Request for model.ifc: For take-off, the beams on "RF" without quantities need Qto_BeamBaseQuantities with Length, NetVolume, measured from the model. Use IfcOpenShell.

First a look at what the model holds.

```python
import ifcopenshell
import ifcopenshell.util.element
import ifcopenshell.util.unit

model = ifcopenshell.open("model.ifc")
print(model.schema)
for unit_type in ("LENGTHUNIT", "AREAUNIT", "VOLUMEUNIT"):
    print(unit_type, ifcopenshell.util.unit.calculate_unit_scale(model, unit_type))
storey = next(s for s in model.by_type("IfcBuildingStorey") if s.Name == "RF")
beams = [e for e in ifcopenshell.util.element.get_decomposition(storey) if e.is_a("IfcBeam")]
for e in sorted(beams, key=lambda e: e.id()):
    print(e.id(), e.is_a(), e.Name, list(ifcopenshell.util.element.get_psets(e, qtos_only=True)), sep=" | ")
```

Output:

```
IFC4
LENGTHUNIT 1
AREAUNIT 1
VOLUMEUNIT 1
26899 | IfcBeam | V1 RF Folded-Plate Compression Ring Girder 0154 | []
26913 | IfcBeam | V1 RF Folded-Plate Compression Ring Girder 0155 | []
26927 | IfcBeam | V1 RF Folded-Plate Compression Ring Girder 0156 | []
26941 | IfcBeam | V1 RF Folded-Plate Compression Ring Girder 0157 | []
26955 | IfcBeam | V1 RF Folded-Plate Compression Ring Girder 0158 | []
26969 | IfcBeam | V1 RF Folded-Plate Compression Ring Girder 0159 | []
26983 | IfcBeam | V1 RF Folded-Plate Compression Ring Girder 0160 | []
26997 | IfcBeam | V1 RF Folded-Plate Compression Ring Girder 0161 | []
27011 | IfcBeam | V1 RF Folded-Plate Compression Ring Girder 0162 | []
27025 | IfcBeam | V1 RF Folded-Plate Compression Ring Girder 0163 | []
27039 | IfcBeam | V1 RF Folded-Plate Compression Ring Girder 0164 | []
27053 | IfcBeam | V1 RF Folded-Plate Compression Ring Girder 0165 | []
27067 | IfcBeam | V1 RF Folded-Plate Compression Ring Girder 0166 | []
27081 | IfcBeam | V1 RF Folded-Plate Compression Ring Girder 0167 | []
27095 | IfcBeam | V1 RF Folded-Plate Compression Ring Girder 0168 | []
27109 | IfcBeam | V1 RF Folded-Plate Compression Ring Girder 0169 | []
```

```python
import ifcopenshell
import ifcopenshell.api.pset
import ifcopenshell.geom
import ifcopenshell.util.element
import ifcopenshell.util.shape
import ifcopenshell.util.unit

model = ifcopenshell.open("model.ifc")
unit_scale = ifcopenshell.util.unit.calculate_unit_scale(model)
volume_scale = ifcopenshell.util.unit.calculate_unit_scale(model, "VOLUMEUNIT")
settings = ifcopenshell.geom.settings()

storey = next(s for s in model.by_type("IfcBuildingStorey") if s.Name == "RF")
beams = [e for e in ifcopenshell.util.element.get_decomposition(storey) if e.is_a("IfcBeam")]

for e in sorted(beams, key=lambda e: e.id()):
    if ifcopenshell.util.element.get_psets(e, qtos_only=True, should_inherit=False):
        continue
    # Geometry comes back in metres, in the element's own axes.
    shape = ifcopenshell.geom.create_shape(settings, e)
    values = {
        "Length": ifcopenshell.util.shape.get_max_xyz(shape.geometry) / unit_scale,
        "NetVolume": ifcopenshell.util.shape.get_volume(shape.geometry) / volume_scale,
    }
    qto = ifcopenshell.api.pset.add_qto(model, product=e, name="Qto_BeamBaseQuantities")
    ifcopenshell.api.pset.edit_qto(model, qto=qto, properties=values)
    print(e.id(), {k: round(v, 3) for k, v in values.items()})

model.write("model_v2.ifc")
```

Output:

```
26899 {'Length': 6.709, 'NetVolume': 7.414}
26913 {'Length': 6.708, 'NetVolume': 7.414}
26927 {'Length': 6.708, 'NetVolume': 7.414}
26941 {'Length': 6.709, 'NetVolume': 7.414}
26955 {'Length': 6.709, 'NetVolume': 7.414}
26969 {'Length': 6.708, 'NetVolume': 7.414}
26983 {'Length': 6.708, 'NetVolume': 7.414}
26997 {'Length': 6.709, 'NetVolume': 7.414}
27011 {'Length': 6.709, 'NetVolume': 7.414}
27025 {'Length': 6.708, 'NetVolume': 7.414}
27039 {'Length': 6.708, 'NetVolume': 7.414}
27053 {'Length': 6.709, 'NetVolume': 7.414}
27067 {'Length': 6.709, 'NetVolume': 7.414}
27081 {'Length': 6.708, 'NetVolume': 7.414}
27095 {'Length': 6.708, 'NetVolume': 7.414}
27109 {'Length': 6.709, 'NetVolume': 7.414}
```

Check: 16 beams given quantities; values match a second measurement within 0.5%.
